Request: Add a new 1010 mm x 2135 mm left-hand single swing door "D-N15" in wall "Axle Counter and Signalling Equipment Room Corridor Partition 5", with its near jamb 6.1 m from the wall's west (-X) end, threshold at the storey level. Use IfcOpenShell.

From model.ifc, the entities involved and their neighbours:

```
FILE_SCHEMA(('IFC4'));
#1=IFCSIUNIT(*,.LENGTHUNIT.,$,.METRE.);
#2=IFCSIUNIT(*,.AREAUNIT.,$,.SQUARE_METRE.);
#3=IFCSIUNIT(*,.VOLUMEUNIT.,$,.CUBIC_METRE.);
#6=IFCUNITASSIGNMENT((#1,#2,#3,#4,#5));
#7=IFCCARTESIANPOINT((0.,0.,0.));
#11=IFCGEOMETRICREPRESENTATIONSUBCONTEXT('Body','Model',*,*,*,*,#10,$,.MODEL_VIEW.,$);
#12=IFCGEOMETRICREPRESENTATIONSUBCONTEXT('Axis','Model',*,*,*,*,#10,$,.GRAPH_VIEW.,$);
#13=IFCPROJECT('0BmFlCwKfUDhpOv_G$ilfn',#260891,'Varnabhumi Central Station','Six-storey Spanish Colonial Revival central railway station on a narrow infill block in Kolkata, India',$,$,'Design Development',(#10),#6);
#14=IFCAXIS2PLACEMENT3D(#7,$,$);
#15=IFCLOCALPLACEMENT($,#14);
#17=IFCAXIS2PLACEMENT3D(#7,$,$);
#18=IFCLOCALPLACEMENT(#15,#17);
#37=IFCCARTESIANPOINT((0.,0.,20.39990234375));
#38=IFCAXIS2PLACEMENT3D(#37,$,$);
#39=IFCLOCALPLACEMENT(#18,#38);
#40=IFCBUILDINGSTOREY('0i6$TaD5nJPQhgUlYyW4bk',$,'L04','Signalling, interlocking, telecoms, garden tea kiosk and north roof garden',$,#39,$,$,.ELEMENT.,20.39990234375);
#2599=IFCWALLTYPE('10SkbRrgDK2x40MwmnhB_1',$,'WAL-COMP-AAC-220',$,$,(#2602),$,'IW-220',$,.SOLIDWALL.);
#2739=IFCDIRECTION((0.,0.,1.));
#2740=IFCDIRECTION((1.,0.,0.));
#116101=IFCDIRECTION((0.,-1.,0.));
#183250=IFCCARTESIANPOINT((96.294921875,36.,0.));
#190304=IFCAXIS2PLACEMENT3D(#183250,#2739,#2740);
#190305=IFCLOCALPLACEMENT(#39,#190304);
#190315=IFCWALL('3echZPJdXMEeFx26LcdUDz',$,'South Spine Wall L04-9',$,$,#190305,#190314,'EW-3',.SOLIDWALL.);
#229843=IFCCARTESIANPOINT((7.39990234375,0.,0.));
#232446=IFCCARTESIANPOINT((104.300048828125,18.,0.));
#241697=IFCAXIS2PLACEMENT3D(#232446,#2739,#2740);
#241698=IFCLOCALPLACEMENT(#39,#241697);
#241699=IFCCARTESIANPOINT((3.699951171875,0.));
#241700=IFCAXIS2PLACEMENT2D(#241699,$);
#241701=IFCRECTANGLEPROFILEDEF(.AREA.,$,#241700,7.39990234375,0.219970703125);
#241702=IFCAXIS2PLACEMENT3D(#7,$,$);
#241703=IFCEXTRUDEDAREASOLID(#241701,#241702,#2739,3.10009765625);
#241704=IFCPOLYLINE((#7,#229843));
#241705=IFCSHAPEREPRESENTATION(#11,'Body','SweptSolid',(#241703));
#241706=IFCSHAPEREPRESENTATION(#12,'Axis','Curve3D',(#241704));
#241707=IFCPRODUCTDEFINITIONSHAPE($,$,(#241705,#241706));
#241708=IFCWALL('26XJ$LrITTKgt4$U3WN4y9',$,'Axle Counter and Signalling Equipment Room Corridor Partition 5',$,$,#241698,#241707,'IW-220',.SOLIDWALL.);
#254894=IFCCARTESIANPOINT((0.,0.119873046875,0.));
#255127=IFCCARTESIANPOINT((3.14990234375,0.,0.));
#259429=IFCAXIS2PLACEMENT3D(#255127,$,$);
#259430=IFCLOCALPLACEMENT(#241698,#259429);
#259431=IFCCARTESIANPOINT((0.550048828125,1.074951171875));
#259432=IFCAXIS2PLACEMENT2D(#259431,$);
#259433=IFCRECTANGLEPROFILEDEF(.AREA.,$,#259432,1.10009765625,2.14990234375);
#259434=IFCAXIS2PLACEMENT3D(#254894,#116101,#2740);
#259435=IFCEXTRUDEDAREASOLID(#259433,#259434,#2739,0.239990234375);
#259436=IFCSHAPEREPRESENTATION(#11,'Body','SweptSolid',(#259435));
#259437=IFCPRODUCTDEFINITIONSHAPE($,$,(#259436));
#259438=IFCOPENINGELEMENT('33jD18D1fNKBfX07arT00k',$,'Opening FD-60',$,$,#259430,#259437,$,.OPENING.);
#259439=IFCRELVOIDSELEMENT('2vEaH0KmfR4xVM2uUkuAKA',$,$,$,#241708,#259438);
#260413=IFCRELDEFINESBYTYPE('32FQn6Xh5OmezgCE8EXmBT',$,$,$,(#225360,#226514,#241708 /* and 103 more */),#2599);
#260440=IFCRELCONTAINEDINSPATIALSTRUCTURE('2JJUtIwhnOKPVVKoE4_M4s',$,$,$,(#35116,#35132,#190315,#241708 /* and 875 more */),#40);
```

```python
import numpy as np
import ifcopenshell
import ifcopenshell.api.feature
import ifcopenshell.api.geometry
import ifcopenshell.api.root
import ifcopenshell.api.spatial
import ifcopenshell.geom
import ifcopenshell.util.element
import ifcopenshell.util.placement
import ifcopenshell.util.representation
import ifcopenshell.util.shape
import ifcopenshell.util.unit

model = ifcopenshell.open("model.ifc")
unit_scale = ifcopenshell.util.unit.calculate_unit_scale(model)
settings = ifcopenshell.geom.settings()


def volume(element):
    """Net volume in cubic metres, openings subtracted."""
    shape = ifcopenshell.geom.create_shape(settings, element)
    return ifcopenshell.util.shape.get_volume(shape.geometry)


wall = model.by_guid("26XJ$LrITTKgt4$U3WN4y9")
storey = ifcopenshell.util.element.get_container(wall, ifc_class="IfcBuildingStorey")
context = ifcopenshell.util.representation.get_context(model, "Model", "Body", "MODEL_VIEW")
before = volume(wall)

width, height, from_end, sill = 1.01, 2.135, 6.1, 0.0  # metres

# The wall runs along its own X axis, and the end named is its -X end.
wall_shape = ifcopenshell.geom.create_shape(settings, wall)
x, y, z = ifcopenshell.util.shape.get_vertices(wall_shape.geometry).T
start = x.min() + from_end
face, thickness = float(y.min()), float(y.max() - y.min())
wall_matrix = ifcopenshell.util.placement.get_local_placement(wall.ObjectPlacement)
level = ifcopenshell.util.placement.get_local_placement(storey.ObjectPlacement)[2, 3]


def in_wall(x, y):
    """Placement at x, y metres in the wall's axes, at sill height."""
    matrix = wall_matrix.copy()
    matrix[:, 3] = wall_matrix @ np.array([x / unit_scale, y / unit_scale, 0.0, 1.0])
    matrix[2, 3] = level + sill / unit_scale
    return matrix


# Opening: a box that overshoots both wall faces by 50 mm.
opening = ifcopenshell.api.root.create_entity(model, ifc_class="IfcOpeningElement", predefined_type="OPENING")
box = ifcopenshell.api.geometry.add_wall_representation(
    model, context=context, length=width, height=height, thickness=thickness + 0.1
)
ifcopenshell.api.geometry.assign_representation(model, product=opening, representation=box)
ifcopenshell.api.geometry.edit_object_placement(model, product=opening, matrix=in_wall(start, face - 0.05), is_si=False)
ifcopenshell.api.feature.add_feature(model, feature=opening, element=wall)

door = ifcopenshell.api.root.create_entity(model, ifc_class="IfcDoor", name="D-N15", predefined_type="DOOR")
door.OverallWidth, door.OverallHeight = width / unit_scale, height / unit_scale
door.OperationType = "SINGLE_SWING_LEFT"
body = ifcopenshell.api.geometry.add_door_representation(
    model,
    context=context,
    overall_width=door.OverallWidth,
    overall_height=door.OverallHeight,
    operation_type="SINGLE_SWING_LEFT",
    lining_properties={"LiningDepth": thickness / unit_scale, "ThresholdDepth": thickness / unit_scale},
)
ifcopenshell.api.geometry.assign_representation(model, product=door, representation=body)
ifcopenshell.api.spatial.assign_container(model, products=[door], relating_structure=storey)
ifcopenshell.api.feature.add_filling(model, opening=opening, element=door)

# The lining spans the wall, so the door starts at the wall face.
ifcopenshell.api.geometry.edit_object_placement(model, product=door, matrix=in_wall(start, face), is_si=False)

after = volume(wall)

print(f"wall volume {before:.3f} -> {after:.3f} m3")

model.write("model_v2.ifc")
```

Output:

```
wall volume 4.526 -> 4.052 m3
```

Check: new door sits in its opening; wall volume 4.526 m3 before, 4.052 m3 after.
